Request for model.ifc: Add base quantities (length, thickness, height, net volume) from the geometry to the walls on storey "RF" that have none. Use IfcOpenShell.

First a look at what the model holds.

```python
import ifcopenshell
import ifcopenshell.util.element
import ifcopenshell.util.unit

model = ifcopenshell.open("model.ifc")
print(model.schema)
for unit_type in ("LENGTHUNIT", "AREAUNIT", "VOLUMEUNIT"):
    print(unit_type, ifcopenshell.util.unit.calculate_unit_scale(model, unit_type))
storey = next(s for s in model.by_type("IfcBuildingStorey") if s.Name == "RF")
walls = [e for e in ifcopenshell.util.element.get_decomposition(storey) if e.is_a("IfcWall")]
for e in sorted(walls, key=lambda e: e.id()):
    print(e.id(), e.is_a(), e.Name, list(ifcopenshell.util.element.get_psets(e, qtos_only=True)), sep=" | ")
```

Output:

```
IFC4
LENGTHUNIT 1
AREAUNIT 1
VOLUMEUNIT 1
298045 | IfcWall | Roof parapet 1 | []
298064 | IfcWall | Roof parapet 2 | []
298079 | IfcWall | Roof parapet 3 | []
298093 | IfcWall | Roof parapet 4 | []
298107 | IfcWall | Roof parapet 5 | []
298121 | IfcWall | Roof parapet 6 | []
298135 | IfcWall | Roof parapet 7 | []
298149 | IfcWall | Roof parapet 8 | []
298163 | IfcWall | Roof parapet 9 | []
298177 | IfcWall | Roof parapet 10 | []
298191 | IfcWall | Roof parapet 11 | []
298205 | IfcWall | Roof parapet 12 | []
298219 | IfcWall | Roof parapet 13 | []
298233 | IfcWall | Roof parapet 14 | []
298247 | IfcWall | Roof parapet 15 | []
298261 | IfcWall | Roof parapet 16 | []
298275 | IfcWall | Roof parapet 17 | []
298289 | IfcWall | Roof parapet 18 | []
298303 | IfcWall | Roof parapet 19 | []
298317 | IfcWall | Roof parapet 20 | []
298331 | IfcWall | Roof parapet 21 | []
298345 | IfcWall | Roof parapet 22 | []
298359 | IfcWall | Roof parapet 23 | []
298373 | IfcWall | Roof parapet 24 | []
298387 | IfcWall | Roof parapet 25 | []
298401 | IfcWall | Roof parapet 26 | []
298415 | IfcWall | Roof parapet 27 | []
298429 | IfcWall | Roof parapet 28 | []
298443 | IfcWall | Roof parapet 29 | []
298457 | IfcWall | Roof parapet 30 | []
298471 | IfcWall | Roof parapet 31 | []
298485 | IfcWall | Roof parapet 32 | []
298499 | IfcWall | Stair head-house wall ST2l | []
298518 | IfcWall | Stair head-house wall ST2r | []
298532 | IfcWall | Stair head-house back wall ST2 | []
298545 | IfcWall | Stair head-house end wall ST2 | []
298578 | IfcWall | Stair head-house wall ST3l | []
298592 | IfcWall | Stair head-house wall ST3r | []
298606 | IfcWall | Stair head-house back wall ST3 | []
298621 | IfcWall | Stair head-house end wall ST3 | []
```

```python
import ifcopenshell
import ifcopenshell.api.pset
import ifcopenshell.geom
import ifcopenshell.util.element
import ifcopenshell.util.shape
import ifcopenshell.util.unit

model = ifcopenshell.open("model.ifc")
unit_scale = ifcopenshell.util.unit.calculate_unit_scale(model)
volume_scale = ifcopenshell.util.unit.calculate_unit_scale(model, "VOLUMEUNIT")
settings = ifcopenshell.geom.settings()

storey = next(s for s in model.by_type("IfcBuildingStorey") if s.Name == "RF")
walls = [e for e in ifcopenshell.util.element.get_decomposition(storey) if e.is_a("IfcWall")]

for e in sorted(walls, key=lambda e: e.id()):
    if ifcopenshell.util.element.get_psets(e, qtos_only=True, should_inherit=False):
        continue
    # Geometry comes back in metres, in the element's own axes.
    shape = ifcopenshell.geom.create_shape(settings, e)
    values = {
        "Length": ifcopenshell.util.shape.get_x(shape.geometry) / unit_scale,
        "Width": ifcopenshell.util.shape.get_y(shape.geometry) / unit_scale,
        "Height": ifcopenshell.util.shape.get_z(shape.geometry) / unit_scale,
        "NetVolume": ifcopenshell.util.shape.get_volume(shape.geometry) / volume_scale,
    }
    qto = ifcopenshell.api.pset.add_qto(model, product=e, name="Qto_WallBaseQuantities")
    ifcopenshell.api.pset.edit_qto(model, qto=qto, properties=values)
    print(e.id(), {k: round(v, 3) for k, v in values.items()})

model.write("model_edited.ifc")
```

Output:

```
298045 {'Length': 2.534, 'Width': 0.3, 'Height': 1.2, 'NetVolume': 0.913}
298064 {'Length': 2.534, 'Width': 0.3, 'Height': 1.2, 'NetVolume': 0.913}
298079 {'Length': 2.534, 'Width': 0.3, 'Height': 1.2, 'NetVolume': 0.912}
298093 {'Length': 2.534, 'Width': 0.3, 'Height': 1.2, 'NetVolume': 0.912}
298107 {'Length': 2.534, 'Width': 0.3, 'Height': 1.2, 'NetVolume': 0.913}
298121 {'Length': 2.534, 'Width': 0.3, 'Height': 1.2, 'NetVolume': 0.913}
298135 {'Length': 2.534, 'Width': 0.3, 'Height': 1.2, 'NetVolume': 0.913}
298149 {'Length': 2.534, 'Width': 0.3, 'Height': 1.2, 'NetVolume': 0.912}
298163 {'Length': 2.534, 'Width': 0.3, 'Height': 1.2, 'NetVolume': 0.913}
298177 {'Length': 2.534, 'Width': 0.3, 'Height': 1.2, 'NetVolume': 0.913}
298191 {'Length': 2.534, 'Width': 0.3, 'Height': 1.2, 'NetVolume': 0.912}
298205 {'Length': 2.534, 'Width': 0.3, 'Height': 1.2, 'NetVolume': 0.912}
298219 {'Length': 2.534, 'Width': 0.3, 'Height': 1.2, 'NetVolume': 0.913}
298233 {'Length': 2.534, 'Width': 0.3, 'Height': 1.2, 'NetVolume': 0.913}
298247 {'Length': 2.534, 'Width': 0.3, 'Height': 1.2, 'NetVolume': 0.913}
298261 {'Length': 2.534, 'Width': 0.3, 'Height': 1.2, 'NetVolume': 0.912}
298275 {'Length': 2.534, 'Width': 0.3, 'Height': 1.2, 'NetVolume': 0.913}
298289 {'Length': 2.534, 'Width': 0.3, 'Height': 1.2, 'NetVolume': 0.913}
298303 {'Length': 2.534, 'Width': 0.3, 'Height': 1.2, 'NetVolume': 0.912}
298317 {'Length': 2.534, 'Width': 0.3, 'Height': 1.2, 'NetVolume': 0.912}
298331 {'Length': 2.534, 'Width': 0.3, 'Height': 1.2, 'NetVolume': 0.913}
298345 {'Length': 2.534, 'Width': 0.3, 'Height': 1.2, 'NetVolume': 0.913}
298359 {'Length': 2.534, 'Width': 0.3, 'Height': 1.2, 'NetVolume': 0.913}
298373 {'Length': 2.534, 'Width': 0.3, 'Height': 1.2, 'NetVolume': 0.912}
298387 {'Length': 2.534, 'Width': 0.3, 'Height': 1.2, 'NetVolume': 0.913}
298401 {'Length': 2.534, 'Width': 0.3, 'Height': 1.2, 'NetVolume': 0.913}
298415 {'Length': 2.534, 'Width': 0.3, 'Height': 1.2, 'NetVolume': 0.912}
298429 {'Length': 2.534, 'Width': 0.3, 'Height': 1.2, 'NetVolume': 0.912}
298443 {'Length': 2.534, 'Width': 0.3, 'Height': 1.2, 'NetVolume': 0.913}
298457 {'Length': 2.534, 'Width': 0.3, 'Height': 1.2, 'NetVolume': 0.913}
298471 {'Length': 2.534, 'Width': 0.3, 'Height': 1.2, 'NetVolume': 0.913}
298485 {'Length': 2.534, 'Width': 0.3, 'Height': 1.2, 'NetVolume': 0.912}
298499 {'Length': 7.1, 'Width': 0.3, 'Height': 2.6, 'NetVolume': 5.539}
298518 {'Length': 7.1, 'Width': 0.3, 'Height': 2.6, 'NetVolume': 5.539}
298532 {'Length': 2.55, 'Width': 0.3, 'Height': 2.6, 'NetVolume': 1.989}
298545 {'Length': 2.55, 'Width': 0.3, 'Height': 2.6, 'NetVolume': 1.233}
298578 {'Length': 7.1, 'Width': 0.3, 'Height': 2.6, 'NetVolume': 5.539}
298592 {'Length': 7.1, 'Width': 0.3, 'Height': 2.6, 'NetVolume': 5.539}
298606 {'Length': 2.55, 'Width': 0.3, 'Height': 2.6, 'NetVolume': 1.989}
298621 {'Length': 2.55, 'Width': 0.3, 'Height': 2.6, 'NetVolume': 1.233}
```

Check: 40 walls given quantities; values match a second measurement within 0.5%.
